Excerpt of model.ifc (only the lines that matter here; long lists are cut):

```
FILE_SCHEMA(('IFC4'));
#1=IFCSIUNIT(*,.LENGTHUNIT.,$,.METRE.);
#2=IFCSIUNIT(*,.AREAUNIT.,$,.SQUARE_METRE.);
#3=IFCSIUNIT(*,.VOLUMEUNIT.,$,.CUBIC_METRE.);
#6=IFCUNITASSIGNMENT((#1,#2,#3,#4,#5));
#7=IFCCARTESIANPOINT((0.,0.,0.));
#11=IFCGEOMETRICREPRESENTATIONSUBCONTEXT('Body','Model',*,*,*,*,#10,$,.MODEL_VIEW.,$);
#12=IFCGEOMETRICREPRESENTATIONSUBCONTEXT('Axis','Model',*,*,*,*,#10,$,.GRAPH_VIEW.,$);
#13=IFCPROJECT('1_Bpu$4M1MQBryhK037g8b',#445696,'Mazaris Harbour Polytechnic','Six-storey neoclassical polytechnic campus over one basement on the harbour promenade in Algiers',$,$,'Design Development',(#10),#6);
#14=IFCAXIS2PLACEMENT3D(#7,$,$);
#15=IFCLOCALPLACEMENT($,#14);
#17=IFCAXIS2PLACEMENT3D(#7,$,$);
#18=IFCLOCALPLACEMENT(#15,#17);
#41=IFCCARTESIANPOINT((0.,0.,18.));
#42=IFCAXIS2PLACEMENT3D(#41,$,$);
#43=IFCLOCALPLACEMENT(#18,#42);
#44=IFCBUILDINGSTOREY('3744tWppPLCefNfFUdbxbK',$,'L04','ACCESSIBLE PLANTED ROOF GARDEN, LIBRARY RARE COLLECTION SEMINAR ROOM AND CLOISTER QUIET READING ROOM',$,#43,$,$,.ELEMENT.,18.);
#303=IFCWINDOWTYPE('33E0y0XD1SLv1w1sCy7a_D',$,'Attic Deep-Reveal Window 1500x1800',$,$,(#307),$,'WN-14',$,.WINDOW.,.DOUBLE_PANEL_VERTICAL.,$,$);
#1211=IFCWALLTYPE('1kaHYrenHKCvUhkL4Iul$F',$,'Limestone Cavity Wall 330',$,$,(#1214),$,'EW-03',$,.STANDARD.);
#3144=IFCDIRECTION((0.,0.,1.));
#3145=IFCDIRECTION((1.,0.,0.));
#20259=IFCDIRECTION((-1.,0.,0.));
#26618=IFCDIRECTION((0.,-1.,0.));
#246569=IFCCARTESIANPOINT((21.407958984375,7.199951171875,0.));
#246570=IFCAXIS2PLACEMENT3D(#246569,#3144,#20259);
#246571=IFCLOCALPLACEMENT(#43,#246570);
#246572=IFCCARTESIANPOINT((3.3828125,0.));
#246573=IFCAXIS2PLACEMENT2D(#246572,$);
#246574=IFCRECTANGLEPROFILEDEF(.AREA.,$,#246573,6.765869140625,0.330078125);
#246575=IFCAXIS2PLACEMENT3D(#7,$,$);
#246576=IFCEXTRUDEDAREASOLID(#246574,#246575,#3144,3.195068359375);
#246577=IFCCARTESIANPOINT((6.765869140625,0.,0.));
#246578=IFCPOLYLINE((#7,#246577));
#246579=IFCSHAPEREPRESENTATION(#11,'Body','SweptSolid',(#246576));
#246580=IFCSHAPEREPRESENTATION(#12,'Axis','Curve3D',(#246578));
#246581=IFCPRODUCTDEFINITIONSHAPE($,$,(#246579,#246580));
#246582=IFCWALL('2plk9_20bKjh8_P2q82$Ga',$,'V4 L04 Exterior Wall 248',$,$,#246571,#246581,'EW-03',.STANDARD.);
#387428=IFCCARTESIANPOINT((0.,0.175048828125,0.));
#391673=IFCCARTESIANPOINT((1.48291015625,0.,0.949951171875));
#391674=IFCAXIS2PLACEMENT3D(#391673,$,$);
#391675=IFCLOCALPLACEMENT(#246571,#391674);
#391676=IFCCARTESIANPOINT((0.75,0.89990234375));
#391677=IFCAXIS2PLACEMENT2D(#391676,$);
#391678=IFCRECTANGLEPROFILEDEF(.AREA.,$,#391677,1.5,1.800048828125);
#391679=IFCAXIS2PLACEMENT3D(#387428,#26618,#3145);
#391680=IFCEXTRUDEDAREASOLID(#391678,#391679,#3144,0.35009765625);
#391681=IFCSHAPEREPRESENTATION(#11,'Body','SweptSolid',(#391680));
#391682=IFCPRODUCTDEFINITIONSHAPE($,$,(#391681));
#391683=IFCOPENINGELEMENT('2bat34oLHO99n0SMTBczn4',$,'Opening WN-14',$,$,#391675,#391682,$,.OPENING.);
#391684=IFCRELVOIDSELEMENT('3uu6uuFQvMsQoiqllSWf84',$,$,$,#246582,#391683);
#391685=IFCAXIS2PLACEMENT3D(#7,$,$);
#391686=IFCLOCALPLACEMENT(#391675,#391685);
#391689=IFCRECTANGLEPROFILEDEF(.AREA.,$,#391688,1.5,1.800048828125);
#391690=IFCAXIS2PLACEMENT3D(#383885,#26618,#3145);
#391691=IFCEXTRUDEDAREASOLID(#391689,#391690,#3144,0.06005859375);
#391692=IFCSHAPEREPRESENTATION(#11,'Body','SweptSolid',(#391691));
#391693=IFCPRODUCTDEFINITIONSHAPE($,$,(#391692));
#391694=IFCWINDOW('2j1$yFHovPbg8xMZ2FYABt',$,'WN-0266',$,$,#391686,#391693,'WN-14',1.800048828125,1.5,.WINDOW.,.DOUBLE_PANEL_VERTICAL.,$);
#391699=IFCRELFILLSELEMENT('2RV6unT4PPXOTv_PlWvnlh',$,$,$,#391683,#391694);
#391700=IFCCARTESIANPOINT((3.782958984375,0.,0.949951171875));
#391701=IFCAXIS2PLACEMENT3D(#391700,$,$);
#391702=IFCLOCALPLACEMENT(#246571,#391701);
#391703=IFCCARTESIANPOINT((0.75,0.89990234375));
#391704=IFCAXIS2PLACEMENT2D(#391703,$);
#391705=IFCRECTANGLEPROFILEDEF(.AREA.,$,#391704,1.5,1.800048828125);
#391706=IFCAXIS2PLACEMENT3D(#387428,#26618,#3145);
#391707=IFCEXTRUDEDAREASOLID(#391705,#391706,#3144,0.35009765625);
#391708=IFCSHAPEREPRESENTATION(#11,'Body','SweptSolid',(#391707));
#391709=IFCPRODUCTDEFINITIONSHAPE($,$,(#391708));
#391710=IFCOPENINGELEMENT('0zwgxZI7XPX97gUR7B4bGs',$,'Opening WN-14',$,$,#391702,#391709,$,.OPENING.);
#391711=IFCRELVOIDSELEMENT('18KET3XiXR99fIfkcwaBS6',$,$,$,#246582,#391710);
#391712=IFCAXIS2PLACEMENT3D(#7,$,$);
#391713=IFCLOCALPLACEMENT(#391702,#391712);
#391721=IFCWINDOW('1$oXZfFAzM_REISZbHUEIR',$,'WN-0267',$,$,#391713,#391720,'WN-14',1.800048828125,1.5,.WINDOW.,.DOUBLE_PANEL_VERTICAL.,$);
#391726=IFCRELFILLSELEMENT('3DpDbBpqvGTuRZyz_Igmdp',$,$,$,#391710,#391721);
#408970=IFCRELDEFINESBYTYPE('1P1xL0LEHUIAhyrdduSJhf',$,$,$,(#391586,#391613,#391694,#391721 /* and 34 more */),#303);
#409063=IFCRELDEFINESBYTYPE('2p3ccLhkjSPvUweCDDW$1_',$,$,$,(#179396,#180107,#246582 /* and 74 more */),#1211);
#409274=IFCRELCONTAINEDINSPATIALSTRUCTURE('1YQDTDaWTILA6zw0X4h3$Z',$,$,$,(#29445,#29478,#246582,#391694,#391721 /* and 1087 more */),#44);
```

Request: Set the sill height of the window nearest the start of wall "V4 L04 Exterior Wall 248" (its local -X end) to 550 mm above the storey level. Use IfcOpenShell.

```python
import numpy as np
import ifcopenshell
import ifcopenshell.api.geometry
import ifcopenshell.geom
import ifcopenshell.util.element
import ifcopenshell.util.placement
import ifcopenshell.util.shape
import ifcopenshell.util.unit

model = ifcopenshell.open("model.ifc")
unit_scale = ifcopenshell.util.unit.calculate_unit_scale(model)

window = model.by_guid("2j1$yFHovPbg8xMZ2FYABt")
opening = window.FillsVoids[0].RelatingOpeningElement
storey = ifcopenshell.util.element.get_container(window, ifc_class="IfcBuildingStorey")
level = ifcopenshell.util.placement.get_local_placement(storey.ObjectPlacement)[2, 3]

# The opening's origin need not be at the sill, so measure its lowest point.
shape = ifcopenshell.geom.create_shape(ifcopenshell.geom.settings(), opening)
bottom = ifcopenshell.util.shape.get_shape_bottom_elevation(shape, shape.geometry) / unit_scale
dz = level + 0.55 - bottom

shift = np.array([0.0, 0.0, dz])
# The window is placed relative to its opening, so it follows when the opening moves.
matrix = ifcopenshell.util.placement.get_local_placement(opening.ObjectPlacement)
matrix[:3, 3] += shift
ifcopenshell.api.geometry.edit_object_placement(
    model, product=opening, matrix=matrix, is_si=False, should_transform_children=True
)

print(f"moved by {dz * unit_scale:+.3f} m")

model.write("model_rev.ifc")
```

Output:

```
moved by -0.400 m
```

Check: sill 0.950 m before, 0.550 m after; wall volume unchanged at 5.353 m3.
